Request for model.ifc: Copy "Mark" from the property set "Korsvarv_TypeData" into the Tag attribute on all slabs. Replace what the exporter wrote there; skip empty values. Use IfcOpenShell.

First a look at what the model holds.

```python
import ifcopenshell
import ifcopenshell.util.element

model = ifcopenshell.open("model.ifc")
print(model.schema)
slabs = model.by_type("IfcSlab")
print(len(slabs), "slabs")
for e in slabs[:8]:
    source = ifcopenshell.util.element.get_pset(e, "Korsvarv_TypeData", "Mark")
    target = e.Tag
    print(e.id(), repr(source), repr(target), sep=" | ")
```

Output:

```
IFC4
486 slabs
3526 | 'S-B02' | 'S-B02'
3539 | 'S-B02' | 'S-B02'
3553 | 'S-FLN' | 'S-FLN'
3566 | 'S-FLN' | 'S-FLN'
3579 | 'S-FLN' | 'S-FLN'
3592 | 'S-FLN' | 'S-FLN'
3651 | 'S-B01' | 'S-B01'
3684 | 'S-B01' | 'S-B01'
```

```python
import ifcopenshell
import ifcopenshell.util.element

model = ifcopenshell.open("model.ifc")

count = 0
for e in model.by_type("IfcSlab"):
    value = ifcopenshell.util.element.get_pset(e, "Korsvarv_TypeData", "Mark")
    current = e.Tag
    if not value or not value.strip() or current == value:
        continue
    e.Tag = value
    count += 1

print(count, "slabs updated")

model.write("model-out.ifc")
```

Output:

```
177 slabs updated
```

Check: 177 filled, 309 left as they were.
